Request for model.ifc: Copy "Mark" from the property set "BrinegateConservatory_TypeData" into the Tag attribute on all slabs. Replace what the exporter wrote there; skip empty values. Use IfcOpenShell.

First a look at what the model holds.

```python
import ifcopenshell
import ifcopenshell.util.element

model = ifcopenshell.open("model.ifc")
print(model.schema)
slabs = model.by_type("IfcSlab")
print(len(slabs), "slabs")
for e in slabs[:8]:
    source = ifcopenshell.util.element.get_pset(e, "BrinegateConservatory_TypeData", "Mark")
    target = e.Tag
    print(e.id(), repr(source), repr(target), sep=" | ")
```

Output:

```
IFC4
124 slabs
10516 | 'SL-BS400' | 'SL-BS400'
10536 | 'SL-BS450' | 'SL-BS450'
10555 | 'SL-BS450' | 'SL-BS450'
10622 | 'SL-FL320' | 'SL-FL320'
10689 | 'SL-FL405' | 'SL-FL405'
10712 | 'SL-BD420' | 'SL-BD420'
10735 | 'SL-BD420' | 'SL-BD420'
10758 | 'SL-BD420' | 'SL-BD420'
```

```python
import ifcopenshell
import ifcopenshell.util.element

model = ifcopenshell.open("model.ifc")

count = 0
for e in model.by_type("IfcSlab"):
    value = ifcopenshell.util.element.get_pset(e, "BrinegateConservatory_TypeData", "Mark")
    current = e.Tag
    if not value or not value.strip() or current == value:
        continue
    e.Tag = value
    count += 1

print(count, "slabs updated")

model.write("model-out.ifc")
```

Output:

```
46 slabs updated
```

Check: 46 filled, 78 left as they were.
